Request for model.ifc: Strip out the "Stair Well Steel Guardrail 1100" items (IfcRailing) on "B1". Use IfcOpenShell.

First a look at what the model holds.

```python
import ifcopenshell
import ifcopenshell.util.element

model = ifcopenshell.open("model.ifc")
print(model.schema)
storey = next(s for s in model.by_type("IfcBuildingStorey") if s.Name == "B1")
railings = [e for e in ifcopenshell.util.element.get_decomposition(storey) if e.is_a("IfcRailing")]
seen = {}
for e in railings:
    element_type = ifcopenshell.util.element.get_type(e)
    name = element_type.Name if element_type not in (None, e) else None
    seen[name] = seen.get(name, 0) + 1
for name, count in sorted(seen.items(), key=str):
    print(count, "x", name)
```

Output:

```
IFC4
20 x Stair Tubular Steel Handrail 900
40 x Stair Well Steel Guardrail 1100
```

```python
import ifcopenshell
import ifcopenshell.api.root
import ifcopenshell.util.element

model = ifcopenshell.open("model.ifc")

storey = next(s for s in model.by_type("IfcBuildingStorey") if s.Name == "B1")
railings = [e for e in ifcopenshell.util.element.get_decomposition(storey) if e.is_a("IfcRailing")]
targets = [e for e in railings if (t := ifcopenshell.util.element.get_type(e)) not in (None, e) and t.Name == "Stair Well Steel Guardrail 1100"]

for e in targets:
    ifcopenshell.api.root.remove_product(model, product=e)
print(len(targets), "removed")

model.write("model_updated.ifc")
```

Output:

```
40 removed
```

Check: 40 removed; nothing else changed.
